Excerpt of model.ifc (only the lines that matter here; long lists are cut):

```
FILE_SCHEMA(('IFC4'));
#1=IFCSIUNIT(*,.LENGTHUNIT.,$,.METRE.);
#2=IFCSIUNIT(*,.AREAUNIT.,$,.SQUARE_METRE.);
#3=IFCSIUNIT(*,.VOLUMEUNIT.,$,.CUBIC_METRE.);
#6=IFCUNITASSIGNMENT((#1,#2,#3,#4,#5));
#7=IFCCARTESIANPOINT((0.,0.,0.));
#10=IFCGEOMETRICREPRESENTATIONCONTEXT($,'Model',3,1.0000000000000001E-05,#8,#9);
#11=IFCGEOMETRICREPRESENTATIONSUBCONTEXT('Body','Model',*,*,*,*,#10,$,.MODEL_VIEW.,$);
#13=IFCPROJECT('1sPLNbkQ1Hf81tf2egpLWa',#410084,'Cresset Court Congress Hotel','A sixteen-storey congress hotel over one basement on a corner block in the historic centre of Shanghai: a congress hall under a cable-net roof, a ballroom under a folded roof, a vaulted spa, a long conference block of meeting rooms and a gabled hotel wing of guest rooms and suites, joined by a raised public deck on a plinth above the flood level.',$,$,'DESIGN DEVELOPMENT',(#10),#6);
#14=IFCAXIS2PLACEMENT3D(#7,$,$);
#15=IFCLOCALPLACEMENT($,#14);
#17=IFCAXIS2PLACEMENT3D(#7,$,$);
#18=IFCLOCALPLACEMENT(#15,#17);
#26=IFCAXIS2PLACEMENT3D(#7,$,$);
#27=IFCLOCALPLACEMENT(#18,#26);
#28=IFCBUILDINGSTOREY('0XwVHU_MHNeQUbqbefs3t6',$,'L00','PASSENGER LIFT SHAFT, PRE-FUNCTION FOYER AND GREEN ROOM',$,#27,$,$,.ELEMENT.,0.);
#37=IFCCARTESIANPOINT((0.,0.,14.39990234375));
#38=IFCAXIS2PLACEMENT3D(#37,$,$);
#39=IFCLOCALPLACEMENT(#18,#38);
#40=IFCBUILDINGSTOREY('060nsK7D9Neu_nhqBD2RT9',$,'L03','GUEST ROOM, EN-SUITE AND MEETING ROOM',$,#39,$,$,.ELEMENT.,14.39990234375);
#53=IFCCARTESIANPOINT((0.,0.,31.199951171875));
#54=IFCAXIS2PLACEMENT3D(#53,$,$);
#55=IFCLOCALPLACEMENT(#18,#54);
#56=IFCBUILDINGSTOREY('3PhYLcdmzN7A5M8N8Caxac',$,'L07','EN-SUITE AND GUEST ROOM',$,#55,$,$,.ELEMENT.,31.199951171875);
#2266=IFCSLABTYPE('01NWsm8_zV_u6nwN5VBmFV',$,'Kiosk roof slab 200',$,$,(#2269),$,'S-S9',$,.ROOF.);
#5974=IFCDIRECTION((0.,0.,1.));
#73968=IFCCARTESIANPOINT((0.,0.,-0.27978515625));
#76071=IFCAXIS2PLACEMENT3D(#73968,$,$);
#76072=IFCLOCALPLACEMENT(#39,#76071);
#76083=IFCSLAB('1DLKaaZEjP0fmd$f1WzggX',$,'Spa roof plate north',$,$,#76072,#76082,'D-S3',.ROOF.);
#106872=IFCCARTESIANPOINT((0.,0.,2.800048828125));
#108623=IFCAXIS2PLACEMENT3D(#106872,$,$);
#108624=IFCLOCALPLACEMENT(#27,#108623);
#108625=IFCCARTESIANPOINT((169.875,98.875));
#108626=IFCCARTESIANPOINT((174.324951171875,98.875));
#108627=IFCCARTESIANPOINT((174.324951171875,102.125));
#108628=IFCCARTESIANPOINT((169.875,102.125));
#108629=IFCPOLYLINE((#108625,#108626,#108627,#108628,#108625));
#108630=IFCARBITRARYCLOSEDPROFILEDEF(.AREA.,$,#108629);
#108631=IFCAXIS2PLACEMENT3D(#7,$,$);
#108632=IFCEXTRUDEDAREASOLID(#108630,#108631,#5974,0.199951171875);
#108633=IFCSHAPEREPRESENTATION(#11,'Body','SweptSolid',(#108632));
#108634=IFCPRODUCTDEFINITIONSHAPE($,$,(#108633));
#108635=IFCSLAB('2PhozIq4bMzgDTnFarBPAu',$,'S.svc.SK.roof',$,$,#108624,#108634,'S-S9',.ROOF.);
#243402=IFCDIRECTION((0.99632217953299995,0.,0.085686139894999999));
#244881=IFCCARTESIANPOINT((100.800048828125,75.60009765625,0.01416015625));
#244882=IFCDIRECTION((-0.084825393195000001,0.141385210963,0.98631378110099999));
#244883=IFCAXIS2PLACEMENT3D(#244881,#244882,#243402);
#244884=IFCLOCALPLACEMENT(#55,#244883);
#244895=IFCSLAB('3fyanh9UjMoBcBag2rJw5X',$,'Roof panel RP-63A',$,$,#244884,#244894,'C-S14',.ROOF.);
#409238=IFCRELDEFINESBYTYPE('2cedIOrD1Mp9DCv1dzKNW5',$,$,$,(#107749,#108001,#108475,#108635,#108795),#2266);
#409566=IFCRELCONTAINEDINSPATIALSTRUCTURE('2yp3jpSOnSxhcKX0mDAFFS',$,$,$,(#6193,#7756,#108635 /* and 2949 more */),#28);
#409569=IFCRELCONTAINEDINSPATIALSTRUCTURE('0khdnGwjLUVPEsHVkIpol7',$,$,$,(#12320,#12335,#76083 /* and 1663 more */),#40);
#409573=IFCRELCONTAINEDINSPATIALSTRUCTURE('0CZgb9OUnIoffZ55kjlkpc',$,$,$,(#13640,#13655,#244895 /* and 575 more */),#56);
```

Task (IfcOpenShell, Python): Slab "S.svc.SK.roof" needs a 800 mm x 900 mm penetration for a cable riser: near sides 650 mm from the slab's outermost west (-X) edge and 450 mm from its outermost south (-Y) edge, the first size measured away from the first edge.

```python
import numpy as np
import ifcopenshell
import ifcopenshell.api.feature
import ifcopenshell.api.geometry
import ifcopenshell.api.root
import ifcopenshell.geom
import ifcopenshell.util.placement
import ifcopenshell.util.representation
import ifcopenshell.util.shape
import ifcopenshell.util.unit

model = ifcopenshell.open("model.ifc")
unit_scale = ifcopenshell.util.unit.calculate_unit_scale(model)
settings = ifcopenshell.geom.settings()


def volume(element):
    """Net volume in cubic metres, openings subtracted."""
    shape = ifcopenshell.geom.create_shape(settings, element)
    return ifcopenshell.util.shape.get_volume(shape.geometry)


slab = model.by_guid("2PhozIq4bMzgDTnFarBPAu")
before = volume(slab)

# Extent in the slab's own axes, in metres. The edges named are its -X and -Y sides.
slab_shape = ifcopenshell.geom.create_shape(settings, slab)
vertices = ifcopenshell.util.shape.get_vertices(slab_shape.geometry)
x_min, y_min, bottom = vertices.min(axis=0)
top = vertices[:, 2].max()

opening = ifcopenshell.api.root.create_entity(model, ifc_class="IfcOpeningElement", name="Cable riser opening", predefined_type="OPENING")
context = ifcopenshell.util.representation.get_context(model, "Model", "Body", "MODEL_VIEW")
width, depth = 0.8, 0.9
outline = [(0.0, 0.0), (width, 0.0), (width, depth), (0.0, depth), (0.0, 0.0)]
# Overshoot both faces by 50 mm so the cut is clean.
shape = ifcopenshell.api.geometry.add_slab_representation(
    model, context=context, depth=top - bottom + 0.1, polyline=outline
)
ifcopenshell.api.geometry.assign_representation(model, product=opening, representation=shape)

matrix = ifcopenshell.util.placement.get_local_placement(slab.ObjectPlacement)
matrix[:, 3] = matrix @ np.append(np.array([x_min + 0.65, y_min + 0.45, bottom - 0.05]) / unit_scale, 1.0)
ifcopenshell.api.geometry.edit_object_placement(model, product=opening, matrix=matrix, is_si=False)
ifcopenshell.api.feature.add_feature(model, feature=opening, element=slab)

after = volume(slab)

print(f"slab volume {before:.3f} -> {after:.3f} m3")

model.write("model_edited.ifc")
```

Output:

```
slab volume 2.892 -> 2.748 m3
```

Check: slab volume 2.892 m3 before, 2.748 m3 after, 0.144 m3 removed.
